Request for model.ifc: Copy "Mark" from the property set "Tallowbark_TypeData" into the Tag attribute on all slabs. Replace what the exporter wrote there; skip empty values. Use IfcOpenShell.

First a look at what the model holds.

```python
import ifcopenshell
import ifcopenshell.util.element

model = ifcopenshell.open("model.ifc")
print(model.schema)
slabs = model.by_type("IfcSlab")
print(len(slabs), "slabs")
for e in slabs[:8]:
    source = ifcopenshell.util.element.get_pset(e, "Tallowbark_TypeData", "Mark")
    target = e.Tag
    print(e.id(), repr(source), repr(target), sep=" | ")
```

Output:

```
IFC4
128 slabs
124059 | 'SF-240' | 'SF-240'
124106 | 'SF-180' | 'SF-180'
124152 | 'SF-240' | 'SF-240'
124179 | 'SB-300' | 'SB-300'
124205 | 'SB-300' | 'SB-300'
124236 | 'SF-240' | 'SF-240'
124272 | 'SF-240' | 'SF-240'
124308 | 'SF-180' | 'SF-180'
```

```python
import ifcopenshell
import ifcopenshell.util.element

model = ifcopenshell.open("model.ifc")

count = 0
for e in model.by_type("IfcSlab"):
    value = ifcopenshell.util.element.get_pset(e, "Tallowbark_TypeData", "Mark")
    current = e.Tag
    if not value or not value.strip() or current == value:
        continue
    e.Tag = value
    count += 1

print(count, "slabs updated")

model.write("model_updated.ifc")
```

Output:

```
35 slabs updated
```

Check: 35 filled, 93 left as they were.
